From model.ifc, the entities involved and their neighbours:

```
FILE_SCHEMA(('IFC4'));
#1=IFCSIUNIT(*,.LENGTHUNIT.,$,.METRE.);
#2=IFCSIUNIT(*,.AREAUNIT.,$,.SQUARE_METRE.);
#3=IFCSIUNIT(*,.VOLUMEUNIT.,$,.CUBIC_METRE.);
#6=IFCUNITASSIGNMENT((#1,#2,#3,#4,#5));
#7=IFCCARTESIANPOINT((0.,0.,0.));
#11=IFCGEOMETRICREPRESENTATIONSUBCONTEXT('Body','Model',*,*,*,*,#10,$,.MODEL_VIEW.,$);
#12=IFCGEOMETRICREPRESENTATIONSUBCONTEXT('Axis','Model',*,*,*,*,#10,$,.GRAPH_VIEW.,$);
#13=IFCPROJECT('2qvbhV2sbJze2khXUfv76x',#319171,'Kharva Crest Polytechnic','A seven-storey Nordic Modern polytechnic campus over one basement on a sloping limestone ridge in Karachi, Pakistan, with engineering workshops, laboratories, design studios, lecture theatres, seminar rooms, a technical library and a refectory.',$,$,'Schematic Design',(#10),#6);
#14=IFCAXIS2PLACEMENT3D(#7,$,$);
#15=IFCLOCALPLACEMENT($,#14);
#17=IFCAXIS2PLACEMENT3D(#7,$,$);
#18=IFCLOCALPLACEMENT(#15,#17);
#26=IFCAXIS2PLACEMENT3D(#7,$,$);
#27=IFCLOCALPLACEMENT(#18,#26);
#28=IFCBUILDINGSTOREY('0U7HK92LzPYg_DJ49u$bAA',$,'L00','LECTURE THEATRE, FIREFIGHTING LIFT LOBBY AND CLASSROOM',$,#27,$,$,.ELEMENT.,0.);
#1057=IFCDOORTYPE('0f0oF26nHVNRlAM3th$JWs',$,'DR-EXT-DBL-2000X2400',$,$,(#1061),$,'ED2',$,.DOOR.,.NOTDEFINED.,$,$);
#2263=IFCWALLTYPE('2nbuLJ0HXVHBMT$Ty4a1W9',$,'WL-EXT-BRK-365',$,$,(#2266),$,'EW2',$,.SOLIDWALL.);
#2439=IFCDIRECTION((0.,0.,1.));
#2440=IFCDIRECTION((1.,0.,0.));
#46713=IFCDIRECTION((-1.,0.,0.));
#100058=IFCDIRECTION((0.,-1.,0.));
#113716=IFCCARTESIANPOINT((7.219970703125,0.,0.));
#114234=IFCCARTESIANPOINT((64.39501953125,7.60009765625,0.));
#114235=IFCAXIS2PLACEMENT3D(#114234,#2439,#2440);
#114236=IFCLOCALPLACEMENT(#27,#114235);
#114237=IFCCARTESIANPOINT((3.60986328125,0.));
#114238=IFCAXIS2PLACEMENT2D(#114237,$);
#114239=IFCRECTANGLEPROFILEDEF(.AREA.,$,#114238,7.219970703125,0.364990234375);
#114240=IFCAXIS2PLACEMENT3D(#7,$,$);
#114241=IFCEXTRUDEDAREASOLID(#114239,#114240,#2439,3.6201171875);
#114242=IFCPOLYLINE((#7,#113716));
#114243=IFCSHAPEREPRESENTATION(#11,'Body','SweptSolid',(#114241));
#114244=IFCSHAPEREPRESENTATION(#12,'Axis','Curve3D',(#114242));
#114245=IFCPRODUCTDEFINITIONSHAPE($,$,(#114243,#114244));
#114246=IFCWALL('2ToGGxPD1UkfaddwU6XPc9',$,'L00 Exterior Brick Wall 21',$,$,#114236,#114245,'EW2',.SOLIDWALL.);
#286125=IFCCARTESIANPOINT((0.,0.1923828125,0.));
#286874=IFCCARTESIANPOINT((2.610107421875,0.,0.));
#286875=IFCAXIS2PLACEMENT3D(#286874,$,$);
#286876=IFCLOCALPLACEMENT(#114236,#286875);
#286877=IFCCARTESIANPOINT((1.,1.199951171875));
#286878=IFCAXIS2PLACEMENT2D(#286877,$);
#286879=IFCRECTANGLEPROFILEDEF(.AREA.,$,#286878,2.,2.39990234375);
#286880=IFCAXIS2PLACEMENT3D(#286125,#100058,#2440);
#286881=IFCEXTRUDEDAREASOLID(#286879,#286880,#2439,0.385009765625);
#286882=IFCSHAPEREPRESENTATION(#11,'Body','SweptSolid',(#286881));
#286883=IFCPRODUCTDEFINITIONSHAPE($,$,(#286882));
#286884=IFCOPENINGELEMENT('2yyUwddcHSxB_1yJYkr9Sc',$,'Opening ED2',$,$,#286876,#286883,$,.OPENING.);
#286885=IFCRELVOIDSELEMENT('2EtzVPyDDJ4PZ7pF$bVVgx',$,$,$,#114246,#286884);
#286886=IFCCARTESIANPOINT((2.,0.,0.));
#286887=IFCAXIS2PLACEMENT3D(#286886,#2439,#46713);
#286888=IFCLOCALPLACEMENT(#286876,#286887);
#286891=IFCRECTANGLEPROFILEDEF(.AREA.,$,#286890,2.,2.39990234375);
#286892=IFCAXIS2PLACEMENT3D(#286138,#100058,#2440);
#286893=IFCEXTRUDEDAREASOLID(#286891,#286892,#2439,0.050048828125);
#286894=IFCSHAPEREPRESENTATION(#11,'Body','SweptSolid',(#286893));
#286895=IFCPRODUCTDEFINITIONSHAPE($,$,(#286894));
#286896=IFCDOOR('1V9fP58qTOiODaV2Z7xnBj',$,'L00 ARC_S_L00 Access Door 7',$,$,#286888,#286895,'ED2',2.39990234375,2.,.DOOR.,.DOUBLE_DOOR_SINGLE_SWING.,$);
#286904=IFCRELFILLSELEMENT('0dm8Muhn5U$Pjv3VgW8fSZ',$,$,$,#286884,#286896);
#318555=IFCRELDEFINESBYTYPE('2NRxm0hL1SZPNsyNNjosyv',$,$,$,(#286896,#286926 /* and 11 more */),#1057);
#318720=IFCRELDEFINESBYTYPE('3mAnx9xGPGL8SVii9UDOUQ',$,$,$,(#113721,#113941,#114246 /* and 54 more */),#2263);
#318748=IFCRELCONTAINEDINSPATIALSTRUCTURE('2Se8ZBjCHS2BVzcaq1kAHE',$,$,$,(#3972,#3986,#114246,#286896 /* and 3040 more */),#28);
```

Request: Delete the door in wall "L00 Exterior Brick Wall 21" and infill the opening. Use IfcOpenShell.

```python
import ifcopenshell
import ifcopenshell.api.feature
import ifcopenshell.api.root
import ifcopenshell.geom
import ifcopenshell.util.shape

model = ifcopenshell.open("model.ifc")
settings = ifcopenshell.geom.settings()


def volume(element):
    """Net volume in cubic metres, openings subtracted."""
    shape = ifcopenshell.geom.create_shape(settings, element)
    return ifcopenshell.util.shape.get_volume(shape.geometry)


door = model.by_guid("1V9fP58qTOiODaV2Z7xnBj")
opening = door.FillsVoids[0].RelatingOpeningElement
wall = opening.VoidsElements[0].RelatingBuildingElement
before = volume(wall)

ifcopenshell.api.root.remove_product(model, product=door)
ifcopenshell.api.feature.remove_feature(model, feature=opening)

after = volume(wall)

print(f"wall volume {before:.3f} -> {after:.3f} m3")

model.write("model-out.ifc")
```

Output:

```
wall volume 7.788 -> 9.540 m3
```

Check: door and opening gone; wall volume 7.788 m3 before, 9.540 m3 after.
